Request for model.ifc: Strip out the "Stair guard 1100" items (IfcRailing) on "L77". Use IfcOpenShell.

First a look at what the model holds.

```python
import ifcopenshell
import ifcopenshell.util.element

model = ifcopenshell.open("model.ifc")
print(model.schema)
storey = next(s for s in model.by_type("IfcBuildingStorey") if s.Name == "L77")
railings = [e for e in ifcopenshell.util.element.get_decomposition(storey) if e.is_a("IfcRailing")]
seen = {}
for e in railings:
    element_type = ifcopenshell.util.element.get_type(e)
    name = element_type.Name if element_type not in (None, e) else None
    seen[name] = seen.get(name, 0) + 1
for name, count in sorted(seen.items(), key=str):
    print(count, "x", name)
```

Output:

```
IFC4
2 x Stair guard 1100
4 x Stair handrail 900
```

```python
import ifcopenshell
import ifcopenshell.api.root
import ifcopenshell.util.element

model = ifcopenshell.open("model.ifc")

storey = next(s for s in model.by_type("IfcBuildingStorey") if s.Name == "L77")
railings = [e for e in ifcopenshell.util.element.get_decomposition(storey) if e.is_a("IfcRailing")]
targets = [e for e in railings if (t := ifcopenshell.util.element.get_type(e)) not in (None, e) and t.Name == "Stair guard 1100"]

for e in targets:
    ifcopenshell.api.root.remove_product(model, product=e)
print(len(targets), "removed")

model.write("model_edited.ifc")
```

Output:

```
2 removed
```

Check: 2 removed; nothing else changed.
